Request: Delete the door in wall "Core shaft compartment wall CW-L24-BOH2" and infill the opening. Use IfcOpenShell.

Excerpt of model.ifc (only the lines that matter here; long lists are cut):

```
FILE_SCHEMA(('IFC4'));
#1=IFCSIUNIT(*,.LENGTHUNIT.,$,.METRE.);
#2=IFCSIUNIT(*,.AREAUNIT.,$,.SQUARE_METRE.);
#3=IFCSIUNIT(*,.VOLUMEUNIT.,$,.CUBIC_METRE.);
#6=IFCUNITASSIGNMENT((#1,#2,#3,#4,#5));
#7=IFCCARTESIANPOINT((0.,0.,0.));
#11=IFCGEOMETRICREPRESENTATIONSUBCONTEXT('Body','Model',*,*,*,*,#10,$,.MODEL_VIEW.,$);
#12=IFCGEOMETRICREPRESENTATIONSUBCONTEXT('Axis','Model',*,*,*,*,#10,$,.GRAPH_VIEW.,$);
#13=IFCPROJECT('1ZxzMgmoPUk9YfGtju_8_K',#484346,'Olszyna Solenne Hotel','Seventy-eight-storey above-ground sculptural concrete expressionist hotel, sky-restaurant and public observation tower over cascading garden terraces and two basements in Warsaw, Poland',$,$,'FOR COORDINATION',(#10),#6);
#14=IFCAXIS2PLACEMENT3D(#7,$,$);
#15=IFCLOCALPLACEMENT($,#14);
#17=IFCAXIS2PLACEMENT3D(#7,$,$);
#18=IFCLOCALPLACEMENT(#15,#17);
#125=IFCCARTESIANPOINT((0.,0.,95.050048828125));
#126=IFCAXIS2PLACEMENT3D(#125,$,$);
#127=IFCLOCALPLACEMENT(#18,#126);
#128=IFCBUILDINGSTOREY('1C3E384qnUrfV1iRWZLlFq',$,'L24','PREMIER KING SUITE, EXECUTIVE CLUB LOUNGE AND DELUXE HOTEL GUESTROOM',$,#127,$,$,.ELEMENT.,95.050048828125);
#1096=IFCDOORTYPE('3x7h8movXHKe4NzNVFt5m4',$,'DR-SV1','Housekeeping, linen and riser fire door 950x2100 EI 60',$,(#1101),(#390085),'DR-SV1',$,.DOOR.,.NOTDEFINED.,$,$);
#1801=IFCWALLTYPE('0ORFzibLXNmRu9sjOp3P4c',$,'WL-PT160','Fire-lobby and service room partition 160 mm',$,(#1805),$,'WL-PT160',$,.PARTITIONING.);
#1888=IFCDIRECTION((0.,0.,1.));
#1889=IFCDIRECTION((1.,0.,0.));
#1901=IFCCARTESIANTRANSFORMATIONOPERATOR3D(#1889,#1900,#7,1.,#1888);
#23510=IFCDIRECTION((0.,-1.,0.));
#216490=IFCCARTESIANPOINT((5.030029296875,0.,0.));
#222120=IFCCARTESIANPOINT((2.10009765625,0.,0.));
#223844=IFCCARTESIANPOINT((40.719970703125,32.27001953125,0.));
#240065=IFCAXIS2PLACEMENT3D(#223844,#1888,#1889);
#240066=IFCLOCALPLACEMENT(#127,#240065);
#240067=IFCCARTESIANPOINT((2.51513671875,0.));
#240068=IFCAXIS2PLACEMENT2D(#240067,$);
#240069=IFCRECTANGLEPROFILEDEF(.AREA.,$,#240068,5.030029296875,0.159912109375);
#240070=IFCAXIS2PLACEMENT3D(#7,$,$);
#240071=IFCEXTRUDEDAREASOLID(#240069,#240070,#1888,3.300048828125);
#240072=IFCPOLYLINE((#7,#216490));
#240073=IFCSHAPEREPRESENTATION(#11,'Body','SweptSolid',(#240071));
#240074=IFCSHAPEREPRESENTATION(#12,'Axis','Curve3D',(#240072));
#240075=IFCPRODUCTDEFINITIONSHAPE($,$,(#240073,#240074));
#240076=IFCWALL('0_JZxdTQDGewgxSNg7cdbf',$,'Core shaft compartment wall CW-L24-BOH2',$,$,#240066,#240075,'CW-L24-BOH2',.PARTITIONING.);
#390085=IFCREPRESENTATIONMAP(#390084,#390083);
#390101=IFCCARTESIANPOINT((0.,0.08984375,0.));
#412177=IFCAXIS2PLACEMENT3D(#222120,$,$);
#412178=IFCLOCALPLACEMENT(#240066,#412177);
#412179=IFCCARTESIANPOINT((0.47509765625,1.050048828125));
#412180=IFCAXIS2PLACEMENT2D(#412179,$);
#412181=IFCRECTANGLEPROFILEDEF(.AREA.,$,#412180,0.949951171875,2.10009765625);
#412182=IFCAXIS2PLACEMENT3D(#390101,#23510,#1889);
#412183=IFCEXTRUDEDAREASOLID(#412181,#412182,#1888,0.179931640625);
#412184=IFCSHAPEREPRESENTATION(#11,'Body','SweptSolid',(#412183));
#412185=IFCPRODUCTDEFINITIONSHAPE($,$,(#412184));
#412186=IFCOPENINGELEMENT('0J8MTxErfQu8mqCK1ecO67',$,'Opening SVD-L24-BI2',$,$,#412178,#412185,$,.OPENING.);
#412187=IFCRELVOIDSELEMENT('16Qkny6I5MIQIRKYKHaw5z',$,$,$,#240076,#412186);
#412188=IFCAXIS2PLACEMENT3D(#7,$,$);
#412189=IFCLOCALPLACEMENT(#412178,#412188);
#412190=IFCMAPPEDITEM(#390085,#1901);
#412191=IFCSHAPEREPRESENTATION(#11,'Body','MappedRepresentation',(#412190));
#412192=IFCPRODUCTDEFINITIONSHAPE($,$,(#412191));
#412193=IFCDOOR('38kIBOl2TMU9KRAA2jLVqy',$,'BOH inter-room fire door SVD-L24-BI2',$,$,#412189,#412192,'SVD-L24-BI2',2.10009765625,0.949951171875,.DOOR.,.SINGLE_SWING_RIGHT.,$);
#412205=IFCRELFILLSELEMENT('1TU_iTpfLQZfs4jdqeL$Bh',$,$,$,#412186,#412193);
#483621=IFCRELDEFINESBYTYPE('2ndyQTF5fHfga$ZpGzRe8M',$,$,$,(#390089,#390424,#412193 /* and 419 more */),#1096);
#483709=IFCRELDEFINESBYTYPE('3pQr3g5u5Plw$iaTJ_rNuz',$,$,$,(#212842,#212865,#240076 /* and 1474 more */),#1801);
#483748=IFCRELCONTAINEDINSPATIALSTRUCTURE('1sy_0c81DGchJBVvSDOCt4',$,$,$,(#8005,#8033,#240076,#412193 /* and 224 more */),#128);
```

```python
import ifcopenshell
import ifcopenshell.api.feature
import ifcopenshell.api.root
import ifcopenshell.geom
import ifcopenshell.util.shape

model = ifcopenshell.open("model.ifc")
settings = ifcopenshell.geom.settings()


def volume(element):
    """Net volume in cubic metres, openings subtracted."""
    shape = ifcopenshell.geom.create_shape(settings, element)
    return ifcopenshell.util.shape.get_volume(shape.geometry)


door = model.by_guid("38kIBOl2TMU9KRAA2jLVqy")
opening = door.FillsVoids[0].RelatingOpeningElement
wall = opening.VoidsElements[0].RelatingBuildingElement
before = volume(wall)

ifcopenshell.api.root.remove_product(model, product=door)
ifcopenshell.api.feature.remove_feature(model, feature=opening)

after = volume(wall)

print(f"wall volume {before:.3f} -> {after:.3f} m3")

model.write("model_rev.ifc")
```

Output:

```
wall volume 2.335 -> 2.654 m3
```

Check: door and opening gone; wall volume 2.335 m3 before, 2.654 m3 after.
